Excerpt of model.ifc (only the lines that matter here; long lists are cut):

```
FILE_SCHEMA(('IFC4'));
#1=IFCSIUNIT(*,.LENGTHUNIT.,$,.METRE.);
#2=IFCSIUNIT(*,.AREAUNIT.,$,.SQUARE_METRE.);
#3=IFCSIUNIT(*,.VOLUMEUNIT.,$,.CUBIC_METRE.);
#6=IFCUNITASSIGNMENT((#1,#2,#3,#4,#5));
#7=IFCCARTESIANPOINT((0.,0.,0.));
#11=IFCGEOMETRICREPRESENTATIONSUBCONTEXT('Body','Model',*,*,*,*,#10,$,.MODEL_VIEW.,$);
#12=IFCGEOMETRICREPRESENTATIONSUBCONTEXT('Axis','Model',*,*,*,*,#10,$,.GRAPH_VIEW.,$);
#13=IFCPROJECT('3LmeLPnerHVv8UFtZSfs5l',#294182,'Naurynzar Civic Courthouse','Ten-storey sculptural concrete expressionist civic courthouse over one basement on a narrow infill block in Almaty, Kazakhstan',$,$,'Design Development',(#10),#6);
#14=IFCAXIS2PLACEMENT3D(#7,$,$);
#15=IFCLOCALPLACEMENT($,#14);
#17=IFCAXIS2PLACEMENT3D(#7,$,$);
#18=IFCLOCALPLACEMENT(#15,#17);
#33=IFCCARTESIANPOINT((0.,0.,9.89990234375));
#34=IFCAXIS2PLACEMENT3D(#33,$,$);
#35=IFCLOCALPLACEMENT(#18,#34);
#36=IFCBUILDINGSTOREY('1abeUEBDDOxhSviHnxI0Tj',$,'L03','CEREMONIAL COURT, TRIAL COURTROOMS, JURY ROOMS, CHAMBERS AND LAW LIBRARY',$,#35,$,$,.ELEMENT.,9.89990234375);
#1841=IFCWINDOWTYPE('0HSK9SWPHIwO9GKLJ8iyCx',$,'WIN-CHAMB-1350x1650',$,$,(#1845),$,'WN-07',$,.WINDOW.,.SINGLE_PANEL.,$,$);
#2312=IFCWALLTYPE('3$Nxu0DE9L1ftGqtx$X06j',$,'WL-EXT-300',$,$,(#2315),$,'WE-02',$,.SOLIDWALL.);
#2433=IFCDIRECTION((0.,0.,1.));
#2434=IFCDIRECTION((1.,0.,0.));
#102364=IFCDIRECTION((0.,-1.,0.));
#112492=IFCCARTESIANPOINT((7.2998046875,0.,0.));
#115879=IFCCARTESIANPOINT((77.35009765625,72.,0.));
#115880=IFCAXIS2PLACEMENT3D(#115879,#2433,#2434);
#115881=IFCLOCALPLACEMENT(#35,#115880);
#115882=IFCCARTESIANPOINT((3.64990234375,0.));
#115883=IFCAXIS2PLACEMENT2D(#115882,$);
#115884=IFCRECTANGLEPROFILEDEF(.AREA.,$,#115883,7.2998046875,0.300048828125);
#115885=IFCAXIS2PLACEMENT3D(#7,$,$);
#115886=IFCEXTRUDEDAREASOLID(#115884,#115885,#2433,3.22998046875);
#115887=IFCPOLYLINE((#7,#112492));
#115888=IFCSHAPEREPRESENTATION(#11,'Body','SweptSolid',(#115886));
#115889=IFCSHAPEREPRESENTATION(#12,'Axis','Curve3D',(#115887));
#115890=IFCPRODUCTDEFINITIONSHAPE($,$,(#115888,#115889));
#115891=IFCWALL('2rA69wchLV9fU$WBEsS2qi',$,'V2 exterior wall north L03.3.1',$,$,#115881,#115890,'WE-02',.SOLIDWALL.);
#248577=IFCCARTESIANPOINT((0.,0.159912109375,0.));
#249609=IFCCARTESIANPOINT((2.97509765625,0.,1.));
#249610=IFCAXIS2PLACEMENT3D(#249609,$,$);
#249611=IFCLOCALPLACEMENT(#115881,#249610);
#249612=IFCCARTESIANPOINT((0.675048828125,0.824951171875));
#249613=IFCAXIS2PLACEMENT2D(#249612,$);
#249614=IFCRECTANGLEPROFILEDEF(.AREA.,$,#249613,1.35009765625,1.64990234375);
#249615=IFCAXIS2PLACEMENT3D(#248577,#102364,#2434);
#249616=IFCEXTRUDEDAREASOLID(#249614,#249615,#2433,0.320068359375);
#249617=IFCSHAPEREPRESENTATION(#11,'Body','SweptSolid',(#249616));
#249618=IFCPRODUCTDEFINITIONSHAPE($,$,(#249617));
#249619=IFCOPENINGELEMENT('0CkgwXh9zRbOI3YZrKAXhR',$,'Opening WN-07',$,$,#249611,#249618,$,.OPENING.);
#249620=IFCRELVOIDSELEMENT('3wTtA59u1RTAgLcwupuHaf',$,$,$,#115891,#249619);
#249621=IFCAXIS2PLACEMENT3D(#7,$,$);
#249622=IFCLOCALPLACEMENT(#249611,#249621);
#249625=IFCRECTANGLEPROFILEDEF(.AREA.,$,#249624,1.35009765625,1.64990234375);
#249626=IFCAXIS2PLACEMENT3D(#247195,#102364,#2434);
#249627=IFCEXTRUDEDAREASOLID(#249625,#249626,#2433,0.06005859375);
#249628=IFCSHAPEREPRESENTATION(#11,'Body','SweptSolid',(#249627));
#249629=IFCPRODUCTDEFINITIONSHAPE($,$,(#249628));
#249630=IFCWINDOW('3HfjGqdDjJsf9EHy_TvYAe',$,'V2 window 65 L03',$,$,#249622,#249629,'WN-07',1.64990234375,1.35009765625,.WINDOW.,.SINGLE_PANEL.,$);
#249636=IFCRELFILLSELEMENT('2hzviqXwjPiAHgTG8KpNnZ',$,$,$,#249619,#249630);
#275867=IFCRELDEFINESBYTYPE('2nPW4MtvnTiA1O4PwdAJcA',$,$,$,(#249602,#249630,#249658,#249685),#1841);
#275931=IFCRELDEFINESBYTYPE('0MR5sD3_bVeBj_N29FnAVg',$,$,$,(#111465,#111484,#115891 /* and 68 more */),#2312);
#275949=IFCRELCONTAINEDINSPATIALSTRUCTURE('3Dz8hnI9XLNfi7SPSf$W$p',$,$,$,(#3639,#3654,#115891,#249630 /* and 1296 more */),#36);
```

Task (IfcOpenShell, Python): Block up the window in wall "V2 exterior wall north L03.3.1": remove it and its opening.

```python
import ifcopenshell
import ifcopenshell.api.feature
import ifcopenshell.api.root
import ifcopenshell.geom
import ifcopenshell.util.shape

model = ifcopenshell.open("model.ifc")
settings = ifcopenshell.geom.settings()


def volume(element):
    """Net volume in cubic metres, openings subtracted."""
    shape = ifcopenshell.geom.create_shape(settings, element)
    return ifcopenshell.util.shape.get_volume(shape.geometry)


window = model.by_guid("3HfjGqdDjJsf9EHy_TvYAe")
opening = window.FillsVoids[0].RelatingOpeningElement
wall = opening.VoidsElements[0].RelatingBuildingElement
before = volume(wall)

ifcopenshell.api.root.remove_product(model, product=window)
ifcopenshell.api.feature.remove_feature(model, feature=opening)

after = volume(wall)

print(f"wall volume {before:.3f} -> {after:.3f} m3")

model.write("model_rev.ifc")
```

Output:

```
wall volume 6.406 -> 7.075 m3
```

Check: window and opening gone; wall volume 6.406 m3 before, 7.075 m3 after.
